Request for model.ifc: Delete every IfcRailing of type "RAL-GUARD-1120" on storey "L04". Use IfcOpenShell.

First a look at what the model holds.

```python
import ifcopenshell
import ifcopenshell.util.element

model = ifcopenshell.open("model.ifc")
print(model.schema)
storey = next(s for s in model.by_type("IfcBuildingStorey") if s.Name == "L04")
railings = [e for e in ifcopenshell.util.element.get_decomposition(storey) if e.is_a("IfcRailing")]
seen = {}
for e in railings:
    element_type = ifcopenshell.util.element.get_type(e)
    name = element_type.Name if element_type not in (None, e) else None
    seen[name] = seen.get(name, 0) + 1
for name, count in sorted(seen.items(), key=str):
    print(count, "x", name)
```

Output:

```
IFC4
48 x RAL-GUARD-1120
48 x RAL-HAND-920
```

```python
import ifcopenshell
import ifcopenshell.api.root
import ifcopenshell.util.element

model = ifcopenshell.open("model.ifc")

storey = next(s for s in model.by_type("IfcBuildingStorey") if s.Name == "L04")
railings = [e for e in ifcopenshell.util.element.get_decomposition(storey) if e.is_a("IfcRailing")]
targets = [e for e in railings if (t := ifcopenshell.util.element.get_type(e)) not in (None, e) and t.Name == "RAL-GUARD-1120"]

for e in targets:
    ifcopenshell.api.root.remove_product(model, product=e)
print(len(targets), "removed")

model.write("model_edited.ifc")
```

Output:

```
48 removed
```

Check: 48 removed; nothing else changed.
